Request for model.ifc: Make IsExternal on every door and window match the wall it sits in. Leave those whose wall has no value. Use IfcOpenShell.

First a look at what the model holds.

```python
import ifcopenshell
import ifcopenshell.util.element

model = ifcopenshell.open("model.ifc")
print(model.schema)
seen = {}
for e in model.by_type("IfcDoor") + model.by_type("IfcWindow"):
    if not e.FillsVoids:
        continue
    host = e.FillsVoids[0].RelatingOpeningElement.VoidsElements[0].RelatingBuildingElement
    own = ifcopenshell.util.element.get_pset(e, f"Pset_{e.is_a()[3:].removesuffix('StandardCase')}Common", "IsExternal")
    wall = ifcopenshell.util.element.get_pset(host, "Pset_WallCommon", "IsExternal")
    seen[e.is_a(), own, wall] = seen.get((e.is_a(), own, wall), 0) + 1
for (cls, own, wall), count in sorted(seen.items(), key=str):
    print(count, cls, "IsExternal:", own, "| host wall:", wall)
```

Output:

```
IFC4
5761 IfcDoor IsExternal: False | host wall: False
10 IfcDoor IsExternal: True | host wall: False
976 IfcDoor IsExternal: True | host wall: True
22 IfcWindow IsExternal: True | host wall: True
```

```python
import ifcopenshell
import ifcopenshell.api.pset
import ifcopenshell.util.element

model = ifcopenshell.open("model.ifc")

count = 0
for ifc_class, pset_name in (("IfcDoor", "Pset_DoorCommon"), ("IfcWindow", "Pset_WindowCommon")):
    for e in model.by_type(ifc_class):
        if not e.FillsVoids:
            continue
        host = e.FillsVoids[0].RelatingOpeningElement.VoidsElements[0].RelatingBuildingElement
        external = ifcopenshell.util.element.get_pset(host, "Pset_WallCommon", "IsExternal")
        if external is None or ifcopenshell.util.element.get_pset(e, pset_name, "IsExternal") == external:
            continue
        pset = ifcopenshell.api.pset.add_pset(model, product=e, name=pset_name)
        ifcopenshell.api.pset.edit_pset(model, pset=pset, properties={"IsExternal": external})
        count += 1

print(count, "updated")

model.write("model_v2.ifc")
```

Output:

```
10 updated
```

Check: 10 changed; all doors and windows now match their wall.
